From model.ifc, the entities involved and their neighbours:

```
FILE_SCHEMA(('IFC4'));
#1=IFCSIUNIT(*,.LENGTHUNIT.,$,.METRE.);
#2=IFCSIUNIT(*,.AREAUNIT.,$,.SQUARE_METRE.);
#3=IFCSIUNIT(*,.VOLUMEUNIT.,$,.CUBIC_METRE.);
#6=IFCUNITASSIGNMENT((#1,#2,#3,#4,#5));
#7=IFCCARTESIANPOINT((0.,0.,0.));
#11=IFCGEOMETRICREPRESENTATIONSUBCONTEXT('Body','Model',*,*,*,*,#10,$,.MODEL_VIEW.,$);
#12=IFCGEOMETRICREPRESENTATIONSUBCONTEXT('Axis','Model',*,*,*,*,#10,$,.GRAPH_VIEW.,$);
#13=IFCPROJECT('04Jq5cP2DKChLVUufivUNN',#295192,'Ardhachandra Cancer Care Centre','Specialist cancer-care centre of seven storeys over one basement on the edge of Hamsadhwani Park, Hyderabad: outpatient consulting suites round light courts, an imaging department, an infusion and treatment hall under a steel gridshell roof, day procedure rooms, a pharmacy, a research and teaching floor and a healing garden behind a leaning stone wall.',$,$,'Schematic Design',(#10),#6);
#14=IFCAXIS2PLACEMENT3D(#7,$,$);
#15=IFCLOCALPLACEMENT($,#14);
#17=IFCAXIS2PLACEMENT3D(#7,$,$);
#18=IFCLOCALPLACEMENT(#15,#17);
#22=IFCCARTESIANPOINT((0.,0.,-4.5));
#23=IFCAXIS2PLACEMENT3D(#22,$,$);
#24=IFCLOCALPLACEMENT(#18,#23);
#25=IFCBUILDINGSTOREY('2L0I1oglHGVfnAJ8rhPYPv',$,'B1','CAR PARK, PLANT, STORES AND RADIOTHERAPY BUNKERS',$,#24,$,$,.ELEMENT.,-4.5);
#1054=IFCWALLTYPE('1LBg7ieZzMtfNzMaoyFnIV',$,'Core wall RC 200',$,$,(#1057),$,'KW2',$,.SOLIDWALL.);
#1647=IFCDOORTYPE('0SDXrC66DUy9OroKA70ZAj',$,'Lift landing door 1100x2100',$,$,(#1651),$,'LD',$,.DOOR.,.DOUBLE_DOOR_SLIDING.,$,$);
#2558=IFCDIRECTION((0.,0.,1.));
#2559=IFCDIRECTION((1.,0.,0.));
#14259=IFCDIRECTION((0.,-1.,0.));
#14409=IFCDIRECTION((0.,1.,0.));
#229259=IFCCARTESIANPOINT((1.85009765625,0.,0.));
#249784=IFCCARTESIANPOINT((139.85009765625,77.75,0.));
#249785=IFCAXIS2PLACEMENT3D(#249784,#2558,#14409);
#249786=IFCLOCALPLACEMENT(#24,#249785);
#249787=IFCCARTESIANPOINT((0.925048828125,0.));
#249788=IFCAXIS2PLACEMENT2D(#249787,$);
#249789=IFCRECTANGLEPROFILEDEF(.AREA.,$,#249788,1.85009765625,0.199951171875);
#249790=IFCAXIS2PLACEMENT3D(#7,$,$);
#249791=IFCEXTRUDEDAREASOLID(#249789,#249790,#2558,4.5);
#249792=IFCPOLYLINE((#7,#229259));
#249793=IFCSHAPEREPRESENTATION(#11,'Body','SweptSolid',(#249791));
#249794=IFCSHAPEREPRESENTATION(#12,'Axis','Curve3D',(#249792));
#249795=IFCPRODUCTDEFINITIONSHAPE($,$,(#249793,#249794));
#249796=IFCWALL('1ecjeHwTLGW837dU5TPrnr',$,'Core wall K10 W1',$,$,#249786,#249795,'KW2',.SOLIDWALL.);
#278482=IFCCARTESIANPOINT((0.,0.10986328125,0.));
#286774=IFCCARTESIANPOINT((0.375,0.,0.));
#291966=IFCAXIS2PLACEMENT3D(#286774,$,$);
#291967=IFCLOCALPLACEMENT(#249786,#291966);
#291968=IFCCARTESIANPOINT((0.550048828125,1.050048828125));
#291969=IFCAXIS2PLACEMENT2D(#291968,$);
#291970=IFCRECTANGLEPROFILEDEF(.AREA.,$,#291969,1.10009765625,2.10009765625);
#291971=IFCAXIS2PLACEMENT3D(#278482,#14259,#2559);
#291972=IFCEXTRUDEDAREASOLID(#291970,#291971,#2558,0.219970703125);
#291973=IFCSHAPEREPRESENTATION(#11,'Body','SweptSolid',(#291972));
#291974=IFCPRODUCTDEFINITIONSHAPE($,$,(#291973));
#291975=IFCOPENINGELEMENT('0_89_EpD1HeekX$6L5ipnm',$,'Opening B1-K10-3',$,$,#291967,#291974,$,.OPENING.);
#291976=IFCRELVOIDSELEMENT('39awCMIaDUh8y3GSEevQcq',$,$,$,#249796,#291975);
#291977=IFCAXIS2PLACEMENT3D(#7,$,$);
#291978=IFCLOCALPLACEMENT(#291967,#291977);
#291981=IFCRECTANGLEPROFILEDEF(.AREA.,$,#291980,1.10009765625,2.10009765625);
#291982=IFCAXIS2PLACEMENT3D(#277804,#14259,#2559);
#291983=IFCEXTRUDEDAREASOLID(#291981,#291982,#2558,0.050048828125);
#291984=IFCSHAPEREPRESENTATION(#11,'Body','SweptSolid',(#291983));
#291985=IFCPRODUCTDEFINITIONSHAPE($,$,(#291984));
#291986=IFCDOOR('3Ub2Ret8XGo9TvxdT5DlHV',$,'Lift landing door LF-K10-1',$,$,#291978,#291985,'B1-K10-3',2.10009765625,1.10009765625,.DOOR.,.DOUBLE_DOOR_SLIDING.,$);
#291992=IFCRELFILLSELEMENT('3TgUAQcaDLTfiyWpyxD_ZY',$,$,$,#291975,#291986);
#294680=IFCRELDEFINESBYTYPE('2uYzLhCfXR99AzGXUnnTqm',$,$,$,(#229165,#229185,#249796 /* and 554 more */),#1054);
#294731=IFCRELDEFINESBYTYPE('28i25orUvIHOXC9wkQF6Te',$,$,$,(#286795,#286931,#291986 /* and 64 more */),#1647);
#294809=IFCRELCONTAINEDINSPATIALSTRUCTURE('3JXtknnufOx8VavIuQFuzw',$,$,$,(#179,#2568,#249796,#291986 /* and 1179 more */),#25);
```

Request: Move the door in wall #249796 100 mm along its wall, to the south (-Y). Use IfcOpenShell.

```python
import ifcopenshell
import ifcopenshell.api.geometry
import ifcopenshell.util.placement

model = ifcopenshell.open("model.ifc")

door = model.by_guid("3Ub2Ret8XGo9TvxdT5DlHV")
opening = door.FillsVoids[0].RelatingOpeningElement
wall = opening.VoidsElements[0].RelatingBuildingElement

wall_matrix = ifcopenshell.util.placement.get_local_placement(wall.ObjectPlacement)
shift = wall_matrix[:3, 0] * -0.1
before = ifcopenshell.util.placement.get_local_placement(door.ObjectPlacement)[:3, 3].copy()

# The door is placed relative to its opening, so it follows when the opening moves.
matrix = ifcopenshell.util.placement.get_local_placement(opening.ObjectPlacement)
matrix[:3, 3] += shift
ifcopenshell.api.geometry.edit_object_placement(
    model, product=opening, matrix=matrix, is_si=False, should_transform_children=True
)

after = ifcopenshell.util.placement.get_local_placement(door.ObjectPlacement)[:3, 3]
print("door moved by", (after - before).round(3) + 0.0)

model.write("model_rev.ifc")
```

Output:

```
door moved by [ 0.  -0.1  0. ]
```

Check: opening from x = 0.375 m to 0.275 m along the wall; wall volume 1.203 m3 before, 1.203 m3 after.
